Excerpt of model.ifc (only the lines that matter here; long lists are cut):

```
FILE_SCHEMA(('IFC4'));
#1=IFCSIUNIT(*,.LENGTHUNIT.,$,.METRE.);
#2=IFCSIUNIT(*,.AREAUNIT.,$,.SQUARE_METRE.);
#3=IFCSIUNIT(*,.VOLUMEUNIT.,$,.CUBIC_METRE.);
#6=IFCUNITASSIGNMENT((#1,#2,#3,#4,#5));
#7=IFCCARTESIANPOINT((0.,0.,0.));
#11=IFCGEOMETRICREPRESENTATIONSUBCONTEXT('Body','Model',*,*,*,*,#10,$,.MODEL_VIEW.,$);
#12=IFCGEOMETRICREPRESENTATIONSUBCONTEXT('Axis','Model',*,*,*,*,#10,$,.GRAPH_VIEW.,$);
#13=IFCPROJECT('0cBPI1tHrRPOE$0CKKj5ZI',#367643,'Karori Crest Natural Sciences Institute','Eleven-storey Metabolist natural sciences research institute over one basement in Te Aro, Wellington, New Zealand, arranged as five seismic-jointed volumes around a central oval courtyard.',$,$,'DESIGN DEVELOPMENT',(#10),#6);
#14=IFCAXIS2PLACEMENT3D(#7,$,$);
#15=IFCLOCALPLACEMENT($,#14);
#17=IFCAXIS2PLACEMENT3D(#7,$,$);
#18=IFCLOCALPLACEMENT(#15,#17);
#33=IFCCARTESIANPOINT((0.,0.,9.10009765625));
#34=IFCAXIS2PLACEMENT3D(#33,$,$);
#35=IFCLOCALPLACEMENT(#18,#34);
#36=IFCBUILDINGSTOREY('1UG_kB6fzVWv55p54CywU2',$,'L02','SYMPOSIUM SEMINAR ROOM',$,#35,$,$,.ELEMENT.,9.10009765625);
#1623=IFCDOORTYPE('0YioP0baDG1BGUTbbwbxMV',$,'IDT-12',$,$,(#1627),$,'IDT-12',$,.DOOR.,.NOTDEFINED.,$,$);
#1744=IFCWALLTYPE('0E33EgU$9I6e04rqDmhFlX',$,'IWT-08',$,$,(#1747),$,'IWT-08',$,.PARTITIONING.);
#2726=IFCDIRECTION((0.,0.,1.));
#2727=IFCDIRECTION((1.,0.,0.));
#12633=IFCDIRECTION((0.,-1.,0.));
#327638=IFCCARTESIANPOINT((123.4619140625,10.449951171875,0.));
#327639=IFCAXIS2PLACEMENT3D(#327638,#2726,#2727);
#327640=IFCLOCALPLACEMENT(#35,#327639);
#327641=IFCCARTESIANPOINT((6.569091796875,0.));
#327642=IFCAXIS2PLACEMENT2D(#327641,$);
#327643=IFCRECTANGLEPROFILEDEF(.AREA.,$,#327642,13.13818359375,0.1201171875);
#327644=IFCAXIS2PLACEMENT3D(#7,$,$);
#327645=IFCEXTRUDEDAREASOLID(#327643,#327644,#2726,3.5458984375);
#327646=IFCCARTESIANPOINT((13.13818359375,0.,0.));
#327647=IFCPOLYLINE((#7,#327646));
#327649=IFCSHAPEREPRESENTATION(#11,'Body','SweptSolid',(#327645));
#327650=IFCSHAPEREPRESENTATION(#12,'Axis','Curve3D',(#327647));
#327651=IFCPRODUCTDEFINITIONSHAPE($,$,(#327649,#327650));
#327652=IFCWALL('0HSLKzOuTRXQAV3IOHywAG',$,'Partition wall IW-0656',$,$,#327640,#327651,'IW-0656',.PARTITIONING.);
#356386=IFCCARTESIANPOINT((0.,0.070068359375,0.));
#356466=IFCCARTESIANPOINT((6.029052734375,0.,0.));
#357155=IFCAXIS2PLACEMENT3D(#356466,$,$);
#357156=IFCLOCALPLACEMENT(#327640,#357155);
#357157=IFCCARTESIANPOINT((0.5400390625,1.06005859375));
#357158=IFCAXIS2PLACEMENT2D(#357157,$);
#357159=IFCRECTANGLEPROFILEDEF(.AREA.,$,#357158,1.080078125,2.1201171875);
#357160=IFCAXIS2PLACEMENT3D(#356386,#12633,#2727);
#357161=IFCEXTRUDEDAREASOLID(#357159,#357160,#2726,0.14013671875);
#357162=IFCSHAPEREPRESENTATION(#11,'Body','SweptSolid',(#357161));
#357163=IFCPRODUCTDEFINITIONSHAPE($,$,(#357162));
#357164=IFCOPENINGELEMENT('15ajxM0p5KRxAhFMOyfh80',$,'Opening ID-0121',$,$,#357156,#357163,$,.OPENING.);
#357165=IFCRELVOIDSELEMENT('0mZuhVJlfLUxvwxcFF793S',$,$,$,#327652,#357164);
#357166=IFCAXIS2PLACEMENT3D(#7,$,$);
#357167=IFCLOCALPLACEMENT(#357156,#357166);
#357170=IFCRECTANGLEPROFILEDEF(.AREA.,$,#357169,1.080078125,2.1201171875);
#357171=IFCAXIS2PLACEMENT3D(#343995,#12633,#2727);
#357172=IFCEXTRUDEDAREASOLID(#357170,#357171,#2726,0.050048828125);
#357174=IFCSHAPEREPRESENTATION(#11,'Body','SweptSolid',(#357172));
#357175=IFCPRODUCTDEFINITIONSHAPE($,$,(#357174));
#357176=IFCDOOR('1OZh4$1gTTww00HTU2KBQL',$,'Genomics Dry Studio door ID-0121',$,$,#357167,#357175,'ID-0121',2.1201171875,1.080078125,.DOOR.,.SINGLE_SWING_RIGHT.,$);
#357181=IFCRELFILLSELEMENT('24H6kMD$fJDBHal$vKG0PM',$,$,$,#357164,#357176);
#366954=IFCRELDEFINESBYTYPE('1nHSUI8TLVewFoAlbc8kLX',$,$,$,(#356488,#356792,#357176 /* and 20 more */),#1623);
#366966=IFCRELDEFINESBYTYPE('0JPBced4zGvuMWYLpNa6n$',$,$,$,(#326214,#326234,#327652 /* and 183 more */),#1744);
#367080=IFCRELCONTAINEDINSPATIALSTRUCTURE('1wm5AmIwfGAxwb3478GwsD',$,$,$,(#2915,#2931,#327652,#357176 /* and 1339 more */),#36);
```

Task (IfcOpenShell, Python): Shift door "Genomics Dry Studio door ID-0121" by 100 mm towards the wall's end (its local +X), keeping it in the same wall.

```python
import ifcopenshell
import ifcopenshell.api.geometry
import ifcopenshell.util.placement

model = ifcopenshell.open("model.ifc")

door = model.by_guid("1OZh4$1gTTww00HTU2KBQL")
opening = door.FillsVoids[0].RelatingOpeningElement
wall = opening.VoidsElements[0].RelatingBuildingElement

wall_matrix = ifcopenshell.util.placement.get_local_placement(wall.ObjectPlacement)
shift = wall_matrix[:3, 0] * 0.1
before = ifcopenshell.util.placement.get_local_placement(door.ObjectPlacement)[:3, 3].copy()

# The door is placed relative to its opening, so it follows when the opening moves.
matrix = ifcopenshell.util.placement.get_local_placement(opening.ObjectPlacement)
matrix[:3, 3] += shift
ifcopenshell.api.geometry.edit_object_placement(
    model, product=opening, matrix=matrix, is_si=False, should_transform_children=True
)

after = ifcopenshell.util.placement.get_local_placement(door.ObjectPlacement)[:3, 3]
print("door moved by", (after - before).round(3) + 0.0)

model.write("model_v2.ifc")
```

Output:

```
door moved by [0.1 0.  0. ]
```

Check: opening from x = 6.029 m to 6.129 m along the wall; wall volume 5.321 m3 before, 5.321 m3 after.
